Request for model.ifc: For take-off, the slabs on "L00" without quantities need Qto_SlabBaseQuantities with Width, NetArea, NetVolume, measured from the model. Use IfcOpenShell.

First a look at what the model holds.

```python
import ifcopenshell
import ifcopenshell.util.element
import ifcopenshell.util.unit

model = ifcopenshell.open("model.ifc")
print(model.schema)
for unit_type in ("LENGTHUNIT", "AREAUNIT", "VOLUMEUNIT"):
    print(unit_type, ifcopenshell.util.unit.calculate_unit_scale(model, unit_type))
storey = next(s for s in model.by_type("IfcBuildingStorey") if s.Name == "L00")
slabs = [e for e in ifcopenshell.util.element.get_decomposition(storey) if e.is_a("IfcSlab")]
for e in sorted(slabs, key=lambda e: e.id()):
    print(e.id(), e.is_a(), e.Name, list(ifcopenshell.util.element.get_psets(e, qtos_only=True)), sep=" | ")
```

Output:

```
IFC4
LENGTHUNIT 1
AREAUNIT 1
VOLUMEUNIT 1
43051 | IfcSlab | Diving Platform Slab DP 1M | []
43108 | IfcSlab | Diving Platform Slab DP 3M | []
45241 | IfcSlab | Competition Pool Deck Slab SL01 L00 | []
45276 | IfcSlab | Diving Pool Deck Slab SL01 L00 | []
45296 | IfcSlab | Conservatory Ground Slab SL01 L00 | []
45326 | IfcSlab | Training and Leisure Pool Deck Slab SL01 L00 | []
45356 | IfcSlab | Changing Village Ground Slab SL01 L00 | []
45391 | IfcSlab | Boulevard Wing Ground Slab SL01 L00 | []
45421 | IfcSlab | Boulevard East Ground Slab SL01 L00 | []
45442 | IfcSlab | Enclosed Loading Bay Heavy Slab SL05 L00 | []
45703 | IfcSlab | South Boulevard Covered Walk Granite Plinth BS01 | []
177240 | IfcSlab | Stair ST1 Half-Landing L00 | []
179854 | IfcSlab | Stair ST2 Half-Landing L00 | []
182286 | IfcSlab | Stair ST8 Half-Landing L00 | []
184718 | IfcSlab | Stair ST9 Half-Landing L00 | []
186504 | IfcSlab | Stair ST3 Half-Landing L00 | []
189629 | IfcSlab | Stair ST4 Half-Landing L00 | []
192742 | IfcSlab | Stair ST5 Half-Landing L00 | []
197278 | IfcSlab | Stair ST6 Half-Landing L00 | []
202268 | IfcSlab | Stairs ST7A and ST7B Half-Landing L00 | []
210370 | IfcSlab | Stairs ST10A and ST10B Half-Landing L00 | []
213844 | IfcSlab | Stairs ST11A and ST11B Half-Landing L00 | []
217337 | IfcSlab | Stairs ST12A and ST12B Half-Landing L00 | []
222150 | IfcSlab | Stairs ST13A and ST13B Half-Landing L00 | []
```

```python
import ifcopenshell
import ifcopenshell.api.pset
import ifcopenshell.geom
import ifcopenshell.util.element
import ifcopenshell.util.shape
import ifcopenshell.util.unit

model = ifcopenshell.open("model.ifc")
unit_scale = ifcopenshell.util.unit.calculate_unit_scale(model)
area_scale = ifcopenshell.util.unit.calculate_unit_scale(model, "AREAUNIT")
volume_scale = ifcopenshell.util.unit.calculate_unit_scale(model, "VOLUMEUNIT")
settings = ifcopenshell.geom.settings()

storey = next(s for s in model.by_type("IfcBuildingStorey") if s.Name == "L00")
slabs = [e for e in ifcopenshell.util.element.get_decomposition(storey) if e.is_a("IfcSlab")]

for e in sorted(slabs, key=lambda e: e.id()):
    if ifcopenshell.util.element.get_psets(e, qtos_only=True, should_inherit=False):
        continue
    # Geometry comes back in metres, in the element's own axes.
    shape = ifcopenshell.geom.create_shape(settings, e)
    values = {
        "Width": ifcopenshell.util.shape.get_z(shape.geometry) / unit_scale,
        "NetArea": ifcopenshell.util.shape.get_footprint_area(shape.geometry) / area_scale,
        "NetVolume": ifcopenshell.util.shape.get_volume(shape.geometry) / volume_scale,
    }
    qto = ifcopenshell.api.pset.add_qto(model, product=e, name="Qto_SlabBaseQuantities")
    ifcopenshell.api.pset.edit_qto(model, qto=qto, properties=values)
    print(e.id(), {k: round(v, 3) for k, v in values.items()})

model.write("model_v2.ifc")
```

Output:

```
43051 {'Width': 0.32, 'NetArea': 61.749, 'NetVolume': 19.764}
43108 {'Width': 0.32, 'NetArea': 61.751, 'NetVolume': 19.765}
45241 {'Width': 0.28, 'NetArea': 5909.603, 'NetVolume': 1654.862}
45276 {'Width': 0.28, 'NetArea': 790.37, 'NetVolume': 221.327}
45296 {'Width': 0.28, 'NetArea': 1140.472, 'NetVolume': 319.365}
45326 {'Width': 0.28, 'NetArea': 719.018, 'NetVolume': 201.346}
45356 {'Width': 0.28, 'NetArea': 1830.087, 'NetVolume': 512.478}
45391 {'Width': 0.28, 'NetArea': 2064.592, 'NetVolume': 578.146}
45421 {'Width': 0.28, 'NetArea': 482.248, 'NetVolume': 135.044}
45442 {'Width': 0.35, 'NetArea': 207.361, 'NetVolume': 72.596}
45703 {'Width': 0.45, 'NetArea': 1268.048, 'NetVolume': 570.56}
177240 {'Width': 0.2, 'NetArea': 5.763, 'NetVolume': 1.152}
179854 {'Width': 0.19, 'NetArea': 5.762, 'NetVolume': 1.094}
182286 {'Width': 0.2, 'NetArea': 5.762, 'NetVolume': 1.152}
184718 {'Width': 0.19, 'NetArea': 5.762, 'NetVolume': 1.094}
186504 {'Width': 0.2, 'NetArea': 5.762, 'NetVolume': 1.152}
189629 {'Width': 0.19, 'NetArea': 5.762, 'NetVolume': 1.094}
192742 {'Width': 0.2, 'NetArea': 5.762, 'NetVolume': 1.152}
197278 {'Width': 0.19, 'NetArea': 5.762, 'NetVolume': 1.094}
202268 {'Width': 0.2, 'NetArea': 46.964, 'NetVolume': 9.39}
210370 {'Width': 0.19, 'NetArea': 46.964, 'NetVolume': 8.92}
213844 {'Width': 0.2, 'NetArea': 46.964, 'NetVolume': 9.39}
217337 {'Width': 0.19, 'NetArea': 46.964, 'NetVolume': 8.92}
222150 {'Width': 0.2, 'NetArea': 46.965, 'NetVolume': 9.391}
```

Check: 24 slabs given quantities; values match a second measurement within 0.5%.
